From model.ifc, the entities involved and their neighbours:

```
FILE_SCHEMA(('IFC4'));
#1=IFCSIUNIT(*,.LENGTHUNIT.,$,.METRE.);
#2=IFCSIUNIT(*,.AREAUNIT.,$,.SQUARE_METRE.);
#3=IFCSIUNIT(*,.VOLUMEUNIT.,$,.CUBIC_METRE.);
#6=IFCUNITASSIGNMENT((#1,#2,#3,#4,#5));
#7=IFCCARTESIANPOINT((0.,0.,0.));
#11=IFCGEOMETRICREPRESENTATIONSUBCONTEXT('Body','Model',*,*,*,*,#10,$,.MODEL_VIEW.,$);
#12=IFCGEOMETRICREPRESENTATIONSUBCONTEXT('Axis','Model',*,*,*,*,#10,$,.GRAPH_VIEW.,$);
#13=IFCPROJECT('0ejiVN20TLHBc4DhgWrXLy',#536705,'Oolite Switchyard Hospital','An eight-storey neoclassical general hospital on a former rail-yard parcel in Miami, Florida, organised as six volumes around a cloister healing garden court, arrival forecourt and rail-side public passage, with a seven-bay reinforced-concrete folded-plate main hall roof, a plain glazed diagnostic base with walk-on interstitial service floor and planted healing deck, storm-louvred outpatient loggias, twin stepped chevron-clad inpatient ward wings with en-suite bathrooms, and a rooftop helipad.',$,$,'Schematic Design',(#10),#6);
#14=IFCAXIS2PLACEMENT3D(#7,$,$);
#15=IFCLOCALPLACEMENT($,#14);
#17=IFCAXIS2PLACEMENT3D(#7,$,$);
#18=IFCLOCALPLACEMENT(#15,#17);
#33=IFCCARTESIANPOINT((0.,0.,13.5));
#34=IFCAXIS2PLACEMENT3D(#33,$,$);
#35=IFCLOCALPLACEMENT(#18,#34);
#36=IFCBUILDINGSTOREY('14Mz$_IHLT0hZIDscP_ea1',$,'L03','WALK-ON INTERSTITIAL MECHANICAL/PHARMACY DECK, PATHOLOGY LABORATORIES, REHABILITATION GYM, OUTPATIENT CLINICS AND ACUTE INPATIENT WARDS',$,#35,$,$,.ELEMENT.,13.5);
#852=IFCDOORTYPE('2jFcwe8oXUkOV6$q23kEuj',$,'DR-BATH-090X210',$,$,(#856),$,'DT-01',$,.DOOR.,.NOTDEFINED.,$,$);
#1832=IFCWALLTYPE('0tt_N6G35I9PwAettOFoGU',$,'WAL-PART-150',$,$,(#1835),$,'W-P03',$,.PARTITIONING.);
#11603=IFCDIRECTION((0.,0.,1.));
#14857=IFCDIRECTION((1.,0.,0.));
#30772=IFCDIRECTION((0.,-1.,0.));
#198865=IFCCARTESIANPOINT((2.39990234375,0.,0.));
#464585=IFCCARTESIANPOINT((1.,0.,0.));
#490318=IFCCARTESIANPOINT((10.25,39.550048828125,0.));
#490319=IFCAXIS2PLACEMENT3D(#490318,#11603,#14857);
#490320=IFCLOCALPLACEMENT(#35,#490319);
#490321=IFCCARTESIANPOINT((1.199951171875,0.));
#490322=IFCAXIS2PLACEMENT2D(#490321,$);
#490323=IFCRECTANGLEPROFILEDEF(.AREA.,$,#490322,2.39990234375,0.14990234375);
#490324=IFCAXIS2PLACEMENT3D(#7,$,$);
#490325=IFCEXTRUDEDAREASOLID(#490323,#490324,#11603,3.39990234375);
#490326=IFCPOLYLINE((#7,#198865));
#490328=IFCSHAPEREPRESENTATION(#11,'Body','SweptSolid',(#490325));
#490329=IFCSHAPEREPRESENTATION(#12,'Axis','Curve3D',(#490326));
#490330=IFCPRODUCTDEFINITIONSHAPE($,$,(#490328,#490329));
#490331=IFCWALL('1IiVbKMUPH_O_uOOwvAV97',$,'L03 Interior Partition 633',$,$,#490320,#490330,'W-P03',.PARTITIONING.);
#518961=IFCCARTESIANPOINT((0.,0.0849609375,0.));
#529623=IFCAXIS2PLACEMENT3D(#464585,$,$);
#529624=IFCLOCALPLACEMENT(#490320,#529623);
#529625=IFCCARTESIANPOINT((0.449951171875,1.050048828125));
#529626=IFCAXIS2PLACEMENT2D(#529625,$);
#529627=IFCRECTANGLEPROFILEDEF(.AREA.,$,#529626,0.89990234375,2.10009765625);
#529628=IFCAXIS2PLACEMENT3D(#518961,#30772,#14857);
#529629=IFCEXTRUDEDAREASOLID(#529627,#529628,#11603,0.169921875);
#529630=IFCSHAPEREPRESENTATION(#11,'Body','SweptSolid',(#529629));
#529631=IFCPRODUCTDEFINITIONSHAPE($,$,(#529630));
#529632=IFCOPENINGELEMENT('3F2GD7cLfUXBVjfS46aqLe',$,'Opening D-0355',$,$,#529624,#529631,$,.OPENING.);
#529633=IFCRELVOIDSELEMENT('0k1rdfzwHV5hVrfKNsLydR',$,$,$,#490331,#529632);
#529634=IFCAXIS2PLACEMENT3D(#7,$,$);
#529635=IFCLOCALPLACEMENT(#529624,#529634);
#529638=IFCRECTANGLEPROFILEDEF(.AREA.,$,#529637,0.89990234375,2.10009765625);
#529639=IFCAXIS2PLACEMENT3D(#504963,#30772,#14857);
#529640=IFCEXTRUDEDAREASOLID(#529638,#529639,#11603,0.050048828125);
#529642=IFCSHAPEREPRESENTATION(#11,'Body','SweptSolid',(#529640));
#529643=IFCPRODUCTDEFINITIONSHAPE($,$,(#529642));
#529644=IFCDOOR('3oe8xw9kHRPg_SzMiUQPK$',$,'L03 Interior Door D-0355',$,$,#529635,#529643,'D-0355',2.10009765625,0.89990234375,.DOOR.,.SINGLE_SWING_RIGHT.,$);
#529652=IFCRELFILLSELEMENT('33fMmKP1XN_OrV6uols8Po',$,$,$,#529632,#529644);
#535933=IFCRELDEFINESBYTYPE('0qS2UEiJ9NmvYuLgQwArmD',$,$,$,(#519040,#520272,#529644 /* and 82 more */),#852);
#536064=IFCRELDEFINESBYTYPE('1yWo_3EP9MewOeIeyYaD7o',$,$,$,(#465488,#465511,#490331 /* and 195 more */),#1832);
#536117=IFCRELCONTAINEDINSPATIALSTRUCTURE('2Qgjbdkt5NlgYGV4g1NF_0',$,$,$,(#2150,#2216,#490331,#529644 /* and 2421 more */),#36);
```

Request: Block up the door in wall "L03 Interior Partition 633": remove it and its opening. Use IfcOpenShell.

```python
import ifcopenshell
import ifcopenshell.api.feature
import ifcopenshell.api.root
import ifcopenshell.geom
import ifcopenshell.util.shape

model = ifcopenshell.open("model.ifc")
settings = ifcopenshell.geom.settings()


def volume(element):
    """Net volume in cubic metres, openings subtracted."""
    shape = ifcopenshell.geom.create_shape(settings, element)
    return ifcopenshell.util.shape.get_volume(shape.geometry)


door = model.by_id(529644)
opening = door.FillsVoids[0].RelatingOpeningElement
wall = opening.VoidsElements[0].RelatingBuildingElement
before = volume(wall)

ifcopenshell.api.root.remove_product(model, product=door)
ifcopenshell.api.feature.remove_feature(model, feature=opening)

after = volume(wall)

print(f"wall volume {before:.3f} -> {after:.3f} m3")

model.write("model-out.ifc")
```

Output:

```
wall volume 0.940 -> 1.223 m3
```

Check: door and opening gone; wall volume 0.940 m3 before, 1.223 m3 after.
